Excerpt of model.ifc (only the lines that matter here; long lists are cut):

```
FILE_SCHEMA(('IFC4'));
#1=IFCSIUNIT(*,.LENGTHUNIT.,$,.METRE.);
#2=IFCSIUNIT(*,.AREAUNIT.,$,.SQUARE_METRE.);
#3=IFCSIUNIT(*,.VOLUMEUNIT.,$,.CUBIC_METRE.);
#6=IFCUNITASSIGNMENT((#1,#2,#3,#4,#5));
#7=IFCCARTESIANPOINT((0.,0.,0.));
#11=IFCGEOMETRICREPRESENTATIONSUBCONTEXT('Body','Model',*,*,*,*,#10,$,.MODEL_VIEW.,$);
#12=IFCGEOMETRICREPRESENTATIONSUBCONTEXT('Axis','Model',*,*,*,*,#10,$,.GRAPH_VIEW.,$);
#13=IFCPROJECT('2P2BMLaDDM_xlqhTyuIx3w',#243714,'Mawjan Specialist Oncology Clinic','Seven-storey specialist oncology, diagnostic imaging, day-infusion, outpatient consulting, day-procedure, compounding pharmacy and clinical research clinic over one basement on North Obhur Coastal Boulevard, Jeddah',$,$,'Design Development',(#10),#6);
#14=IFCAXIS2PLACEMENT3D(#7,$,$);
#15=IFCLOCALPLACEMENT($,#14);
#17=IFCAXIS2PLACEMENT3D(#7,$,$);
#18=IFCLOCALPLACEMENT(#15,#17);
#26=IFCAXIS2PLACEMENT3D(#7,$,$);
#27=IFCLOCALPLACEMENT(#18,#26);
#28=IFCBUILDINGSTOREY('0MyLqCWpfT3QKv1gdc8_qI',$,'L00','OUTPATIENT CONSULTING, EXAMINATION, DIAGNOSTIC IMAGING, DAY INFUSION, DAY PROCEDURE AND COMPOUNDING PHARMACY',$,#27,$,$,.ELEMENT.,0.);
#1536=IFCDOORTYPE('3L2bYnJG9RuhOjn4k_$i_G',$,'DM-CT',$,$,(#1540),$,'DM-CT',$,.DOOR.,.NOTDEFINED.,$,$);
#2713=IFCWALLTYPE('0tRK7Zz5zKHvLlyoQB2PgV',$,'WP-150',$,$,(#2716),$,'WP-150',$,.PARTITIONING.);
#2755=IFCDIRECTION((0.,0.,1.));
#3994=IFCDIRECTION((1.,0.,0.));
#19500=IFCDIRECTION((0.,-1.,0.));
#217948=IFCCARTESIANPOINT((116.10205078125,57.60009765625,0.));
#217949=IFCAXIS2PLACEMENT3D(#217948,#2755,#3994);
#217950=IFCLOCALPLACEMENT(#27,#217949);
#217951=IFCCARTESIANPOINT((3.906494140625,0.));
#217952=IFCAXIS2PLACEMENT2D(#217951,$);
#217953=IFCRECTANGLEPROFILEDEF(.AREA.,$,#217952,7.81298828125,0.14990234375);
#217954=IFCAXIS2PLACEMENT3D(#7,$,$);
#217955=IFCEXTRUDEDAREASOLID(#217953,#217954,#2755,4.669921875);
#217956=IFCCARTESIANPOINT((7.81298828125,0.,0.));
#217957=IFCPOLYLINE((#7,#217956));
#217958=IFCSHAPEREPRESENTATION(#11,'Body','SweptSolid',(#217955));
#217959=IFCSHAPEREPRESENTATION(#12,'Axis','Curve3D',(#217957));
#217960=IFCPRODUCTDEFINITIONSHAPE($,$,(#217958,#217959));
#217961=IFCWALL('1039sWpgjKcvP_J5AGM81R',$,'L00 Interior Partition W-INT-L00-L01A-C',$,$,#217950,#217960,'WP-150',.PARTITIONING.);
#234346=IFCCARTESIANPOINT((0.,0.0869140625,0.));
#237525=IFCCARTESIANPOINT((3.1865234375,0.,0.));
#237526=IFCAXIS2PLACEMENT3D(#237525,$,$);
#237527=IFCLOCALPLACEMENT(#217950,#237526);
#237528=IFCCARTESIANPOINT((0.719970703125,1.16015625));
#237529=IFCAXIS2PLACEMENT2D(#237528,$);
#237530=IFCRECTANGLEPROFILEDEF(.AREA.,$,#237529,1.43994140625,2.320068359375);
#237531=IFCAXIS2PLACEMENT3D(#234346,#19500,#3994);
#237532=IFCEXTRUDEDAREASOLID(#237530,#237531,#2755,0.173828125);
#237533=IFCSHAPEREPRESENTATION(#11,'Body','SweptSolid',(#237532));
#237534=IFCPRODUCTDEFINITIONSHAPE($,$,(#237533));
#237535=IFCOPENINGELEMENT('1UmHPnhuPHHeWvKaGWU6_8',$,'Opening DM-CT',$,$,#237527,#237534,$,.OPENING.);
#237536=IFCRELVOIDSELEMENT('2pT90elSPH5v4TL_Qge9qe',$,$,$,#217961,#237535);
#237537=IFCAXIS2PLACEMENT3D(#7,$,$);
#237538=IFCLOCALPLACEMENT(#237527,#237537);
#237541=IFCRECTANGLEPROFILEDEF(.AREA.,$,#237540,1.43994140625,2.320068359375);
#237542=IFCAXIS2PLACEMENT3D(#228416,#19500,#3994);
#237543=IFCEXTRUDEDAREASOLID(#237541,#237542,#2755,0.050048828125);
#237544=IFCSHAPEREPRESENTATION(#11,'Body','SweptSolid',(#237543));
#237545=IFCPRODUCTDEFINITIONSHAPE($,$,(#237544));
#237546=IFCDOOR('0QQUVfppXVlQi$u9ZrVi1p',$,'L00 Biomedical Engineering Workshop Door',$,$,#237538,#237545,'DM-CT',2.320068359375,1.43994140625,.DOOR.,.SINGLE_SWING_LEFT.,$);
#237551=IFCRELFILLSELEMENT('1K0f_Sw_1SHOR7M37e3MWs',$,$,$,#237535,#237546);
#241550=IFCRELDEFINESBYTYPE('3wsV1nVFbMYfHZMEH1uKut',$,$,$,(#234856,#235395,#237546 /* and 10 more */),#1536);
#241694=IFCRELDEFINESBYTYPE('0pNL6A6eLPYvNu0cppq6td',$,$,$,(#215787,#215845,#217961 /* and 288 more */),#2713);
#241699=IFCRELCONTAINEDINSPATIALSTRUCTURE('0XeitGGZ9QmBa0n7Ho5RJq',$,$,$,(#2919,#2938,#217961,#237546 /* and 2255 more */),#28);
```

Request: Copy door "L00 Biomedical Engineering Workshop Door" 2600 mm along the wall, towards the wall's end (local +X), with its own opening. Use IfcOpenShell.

```python
import ifcopenshell
import ifcopenshell.api.feature
import ifcopenshell.api.geometry
import ifcopenshell.api.root
import ifcopenshell.geom
import ifcopenshell.util.element
import ifcopenshell.util.placement
import ifcopenshell.util.shape

model = ifcopenshell.open("model.ifc")
settings = ifcopenshell.geom.settings()


def volume(element):
    """Net volume in cubic metres, openings subtracted."""
    shape = ifcopenshell.geom.create_shape(settings, element)
    return ifcopenshell.util.shape.get_volume(shape.geometry)


door = model.by_guid("0QQUVfppXVlQi$u9ZrVi1p")
opening = door.FillsVoids[0].RelatingOpeningElement
wall = opening.VoidsElements[0].RelatingBuildingElement
before = volume(wall)
shift = ifcopenshell.util.placement.get_local_placement(wall.ObjectPlacement)[:3, 0] * 2.6

# copy_class copies the void relationship, type, container and properties, but no geometry.
new_opening = ifcopenshell.api.root.copy_class(model, product=opening)
new_opening.Representation = ifcopenshell.util.element.copy_deep(
    model, opening.Representation, exclude=["IfcGeometricRepresentationContext", "IfcRepresentationMap"]
)
new_door = ifcopenshell.api.root.copy_class(model, product=door)
new_door.Representation = ifcopenshell.util.element.copy_deep(
    model, door.Representation, exclude=["IfcGeometricRepresentationContext", "IfcRepresentationMap"]
)
new_door.Tag = None
ifcopenshell.api.feature.add_filling(model, opening=new_opening, element=new_door)

for old, new in ((opening, new_opening), (door, new_door)):
    matrix = ifcopenshell.util.placement.get_local_placement(old.ObjectPlacement)
    matrix[:3, 3] += shift
    ifcopenshell.api.geometry.edit_object_placement(model, product=new, matrix=matrix, is_si=False)

after = volume(wall)

print(f"wall volume {before:.3f} -> {after:.3f} m3")

model.write("model-out.ifc")
```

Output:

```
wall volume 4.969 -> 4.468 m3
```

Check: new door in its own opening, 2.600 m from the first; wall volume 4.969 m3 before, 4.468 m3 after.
